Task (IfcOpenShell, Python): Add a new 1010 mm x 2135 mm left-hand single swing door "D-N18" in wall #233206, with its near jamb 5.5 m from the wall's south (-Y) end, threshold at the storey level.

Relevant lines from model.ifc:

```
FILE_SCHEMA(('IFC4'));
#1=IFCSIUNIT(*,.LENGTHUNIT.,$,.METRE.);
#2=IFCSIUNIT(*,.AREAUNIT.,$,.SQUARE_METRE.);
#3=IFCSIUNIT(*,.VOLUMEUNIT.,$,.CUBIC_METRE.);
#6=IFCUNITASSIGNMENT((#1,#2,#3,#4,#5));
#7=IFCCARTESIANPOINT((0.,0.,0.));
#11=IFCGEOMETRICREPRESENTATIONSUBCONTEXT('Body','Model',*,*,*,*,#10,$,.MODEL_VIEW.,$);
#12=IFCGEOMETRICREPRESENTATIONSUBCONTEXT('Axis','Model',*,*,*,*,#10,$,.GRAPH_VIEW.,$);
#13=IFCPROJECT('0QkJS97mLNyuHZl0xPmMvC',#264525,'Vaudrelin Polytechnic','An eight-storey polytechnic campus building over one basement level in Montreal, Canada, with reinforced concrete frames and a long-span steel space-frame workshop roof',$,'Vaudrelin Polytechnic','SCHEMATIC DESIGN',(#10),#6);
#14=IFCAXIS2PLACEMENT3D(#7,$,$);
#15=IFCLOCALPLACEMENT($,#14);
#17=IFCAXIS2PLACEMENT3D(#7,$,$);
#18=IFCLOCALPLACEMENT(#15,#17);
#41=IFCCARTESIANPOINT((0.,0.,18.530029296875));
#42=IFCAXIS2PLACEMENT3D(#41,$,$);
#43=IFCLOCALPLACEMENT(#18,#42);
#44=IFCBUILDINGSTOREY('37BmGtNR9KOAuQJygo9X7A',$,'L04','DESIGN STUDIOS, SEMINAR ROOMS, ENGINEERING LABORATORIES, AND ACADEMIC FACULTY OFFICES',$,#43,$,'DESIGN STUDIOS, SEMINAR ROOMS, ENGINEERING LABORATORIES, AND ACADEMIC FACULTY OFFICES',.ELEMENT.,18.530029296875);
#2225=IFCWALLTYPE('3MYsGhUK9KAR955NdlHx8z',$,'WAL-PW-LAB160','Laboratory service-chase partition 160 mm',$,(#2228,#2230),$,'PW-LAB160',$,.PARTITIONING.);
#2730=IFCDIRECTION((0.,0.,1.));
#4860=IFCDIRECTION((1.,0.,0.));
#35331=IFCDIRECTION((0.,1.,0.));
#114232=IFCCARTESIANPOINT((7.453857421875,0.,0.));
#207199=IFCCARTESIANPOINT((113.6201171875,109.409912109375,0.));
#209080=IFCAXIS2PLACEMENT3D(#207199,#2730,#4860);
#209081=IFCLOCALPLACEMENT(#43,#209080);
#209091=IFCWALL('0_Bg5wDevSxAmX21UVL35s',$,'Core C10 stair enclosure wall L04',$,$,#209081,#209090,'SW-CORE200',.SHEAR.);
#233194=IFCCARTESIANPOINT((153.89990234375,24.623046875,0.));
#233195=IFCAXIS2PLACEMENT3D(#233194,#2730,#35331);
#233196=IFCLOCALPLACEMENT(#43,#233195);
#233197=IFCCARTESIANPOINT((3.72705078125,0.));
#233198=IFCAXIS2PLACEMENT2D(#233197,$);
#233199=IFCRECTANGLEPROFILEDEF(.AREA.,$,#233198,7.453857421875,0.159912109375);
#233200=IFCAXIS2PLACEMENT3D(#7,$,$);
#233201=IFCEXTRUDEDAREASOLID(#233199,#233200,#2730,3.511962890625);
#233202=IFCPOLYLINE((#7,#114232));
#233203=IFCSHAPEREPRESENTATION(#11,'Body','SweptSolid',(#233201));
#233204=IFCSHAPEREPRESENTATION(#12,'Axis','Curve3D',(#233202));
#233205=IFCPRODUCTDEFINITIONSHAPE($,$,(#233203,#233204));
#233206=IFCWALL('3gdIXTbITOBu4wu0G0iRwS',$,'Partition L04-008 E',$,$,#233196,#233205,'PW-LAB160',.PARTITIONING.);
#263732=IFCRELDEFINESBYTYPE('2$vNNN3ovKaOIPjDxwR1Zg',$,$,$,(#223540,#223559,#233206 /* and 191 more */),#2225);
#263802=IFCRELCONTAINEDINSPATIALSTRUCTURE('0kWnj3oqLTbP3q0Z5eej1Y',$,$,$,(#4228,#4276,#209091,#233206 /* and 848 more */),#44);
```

```python
import numpy as np
import ifcopenshell
import ifcopenshell.api.feature
import ifcopenshell.api.geometry
import ifcopenshell.api.root
import ifcopenshell.api.spatial
import ifcopenshell.geom
import ifcopenshell.util.element
import ifcopenshell.util.placement
import ifcopenshell.util.representation
import ifcopenshell.util.shape
import ifcopenshell.util.unit

model = ifcopenshell.open("model.ifc")
unit_scale = ifcopenshell.util.unit.calculate_unit_scale(model)
settings = ifcopenshell.geom.settings()


def volume(element):
    """Net volume in cubic metres, openings subtracted."""
    shape = ifcopenshell.geom.create_shape(settings, element)
    return ifcopenshell.util.shape.get_volume(shape.geometry)


wall = model.by_guid("3gdIXTbITOBu4wu0G0iRwS")
storey = ifcopenshell.util.element.get_container(wall, ifc_class="IfcBuildingStorey")
context = ifcopenshell.util.representation.get_context(model, "Model", "Body", "MODEL_VIEW")
before = volume(wall)

width, height, from_end, sill = 1.01, 2.135, 5.5, 0.0  # metres

# The wall runs along its own X axis, and the end named is its -X end.
wall_shape = ifcopenshell.geom.create_shape(settings, wall)
x, y, z = ifcopenshell.util.shape.get_vertices(wall_shape.geometry).T
start = x.min() + from_end
face, thickness = float(y.min()), float(y.max() - y.min())
wall_matrix = ifcopenshell.util.placement.get_local_placement(wall.ObjectPlacement)
level = ifcopenshell.util.placement.get_local_placement(storey.ObjectPlacement)[2, 3]


def in_wall(x, y):
    """Placement at x, y metres in the wall's axes, at sill height."""
    matrix = wall_matrix.copy()
    matrix[:, 3] = wall_matrix @ np.array([x / unit_scale, y / unit_scale, 0.0, 1.0])
    matrix[2, 3] = level + sill / unit_scale
    return matrix


# Opening: a box that overshoots both wall faces by 50 mm.
opening = ifcopenshell.api.root.create_entity(model, ifc_class="IfcOpeningElement", predefined_type="OPENING")
box = ifcopenshell.api.geometry.add_wall_representation(
    model, context=context, length=width, height=height, thickness=thickness + 0.1
)
ifcopenshell.api.geometry.assign_representation(model, product=opening, representation=box)
ifcopenshell.api.geometry.edit_object_placement(model, product=opening, matrix=in_wall(start, face - 0.05), is_si=False)
ifcopenshell.api.feature.add_feature(model, feature=opening, element=wall)

door = ifcopenshell.api.root.create_entity(model, ifc_class="IfcDoor", name="D-N18", predefined_type="DOOR")
door.OverallWidth, door.OverallHeight = width / unit_scale, height / unit_scale
door.OperationType = "SINGLE_SWING_LEFT"
body = ifcopenshell.api.geometry.add_door_representation(
    model,
    context=context,
    overall_width=door.OverallWidth,
    overall_height=door.OverallHeight,
    operation_type="SINGLE_SWING_LEFT",
    lining_properties={"LiningDepth": thickness / unit_scale, "ThresholdDepth": thickness / unit_scale},
)
ifcopenshell.api.geometry.assign_representation(model, product=door, representation=body)
ifcopenshell.api.spatial.assign_container(model, products=[door], relating_structure=storey)
ifcopenshell.api.feature.add_filling(model, opening=opening, element=door)

# The lining spans the wall, so the door starts at the wall face.
ifcopenshell.api.geometry.edit_object_placement(model, product=door, matrix=in_wall(start, face), is_si=False)

after = volume(wall)

print(f"wall volume {before:.3f} -> {after:.3f} m3")

model.write("model-out.ifc")
```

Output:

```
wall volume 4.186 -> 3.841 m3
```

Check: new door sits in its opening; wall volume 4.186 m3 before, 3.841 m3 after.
